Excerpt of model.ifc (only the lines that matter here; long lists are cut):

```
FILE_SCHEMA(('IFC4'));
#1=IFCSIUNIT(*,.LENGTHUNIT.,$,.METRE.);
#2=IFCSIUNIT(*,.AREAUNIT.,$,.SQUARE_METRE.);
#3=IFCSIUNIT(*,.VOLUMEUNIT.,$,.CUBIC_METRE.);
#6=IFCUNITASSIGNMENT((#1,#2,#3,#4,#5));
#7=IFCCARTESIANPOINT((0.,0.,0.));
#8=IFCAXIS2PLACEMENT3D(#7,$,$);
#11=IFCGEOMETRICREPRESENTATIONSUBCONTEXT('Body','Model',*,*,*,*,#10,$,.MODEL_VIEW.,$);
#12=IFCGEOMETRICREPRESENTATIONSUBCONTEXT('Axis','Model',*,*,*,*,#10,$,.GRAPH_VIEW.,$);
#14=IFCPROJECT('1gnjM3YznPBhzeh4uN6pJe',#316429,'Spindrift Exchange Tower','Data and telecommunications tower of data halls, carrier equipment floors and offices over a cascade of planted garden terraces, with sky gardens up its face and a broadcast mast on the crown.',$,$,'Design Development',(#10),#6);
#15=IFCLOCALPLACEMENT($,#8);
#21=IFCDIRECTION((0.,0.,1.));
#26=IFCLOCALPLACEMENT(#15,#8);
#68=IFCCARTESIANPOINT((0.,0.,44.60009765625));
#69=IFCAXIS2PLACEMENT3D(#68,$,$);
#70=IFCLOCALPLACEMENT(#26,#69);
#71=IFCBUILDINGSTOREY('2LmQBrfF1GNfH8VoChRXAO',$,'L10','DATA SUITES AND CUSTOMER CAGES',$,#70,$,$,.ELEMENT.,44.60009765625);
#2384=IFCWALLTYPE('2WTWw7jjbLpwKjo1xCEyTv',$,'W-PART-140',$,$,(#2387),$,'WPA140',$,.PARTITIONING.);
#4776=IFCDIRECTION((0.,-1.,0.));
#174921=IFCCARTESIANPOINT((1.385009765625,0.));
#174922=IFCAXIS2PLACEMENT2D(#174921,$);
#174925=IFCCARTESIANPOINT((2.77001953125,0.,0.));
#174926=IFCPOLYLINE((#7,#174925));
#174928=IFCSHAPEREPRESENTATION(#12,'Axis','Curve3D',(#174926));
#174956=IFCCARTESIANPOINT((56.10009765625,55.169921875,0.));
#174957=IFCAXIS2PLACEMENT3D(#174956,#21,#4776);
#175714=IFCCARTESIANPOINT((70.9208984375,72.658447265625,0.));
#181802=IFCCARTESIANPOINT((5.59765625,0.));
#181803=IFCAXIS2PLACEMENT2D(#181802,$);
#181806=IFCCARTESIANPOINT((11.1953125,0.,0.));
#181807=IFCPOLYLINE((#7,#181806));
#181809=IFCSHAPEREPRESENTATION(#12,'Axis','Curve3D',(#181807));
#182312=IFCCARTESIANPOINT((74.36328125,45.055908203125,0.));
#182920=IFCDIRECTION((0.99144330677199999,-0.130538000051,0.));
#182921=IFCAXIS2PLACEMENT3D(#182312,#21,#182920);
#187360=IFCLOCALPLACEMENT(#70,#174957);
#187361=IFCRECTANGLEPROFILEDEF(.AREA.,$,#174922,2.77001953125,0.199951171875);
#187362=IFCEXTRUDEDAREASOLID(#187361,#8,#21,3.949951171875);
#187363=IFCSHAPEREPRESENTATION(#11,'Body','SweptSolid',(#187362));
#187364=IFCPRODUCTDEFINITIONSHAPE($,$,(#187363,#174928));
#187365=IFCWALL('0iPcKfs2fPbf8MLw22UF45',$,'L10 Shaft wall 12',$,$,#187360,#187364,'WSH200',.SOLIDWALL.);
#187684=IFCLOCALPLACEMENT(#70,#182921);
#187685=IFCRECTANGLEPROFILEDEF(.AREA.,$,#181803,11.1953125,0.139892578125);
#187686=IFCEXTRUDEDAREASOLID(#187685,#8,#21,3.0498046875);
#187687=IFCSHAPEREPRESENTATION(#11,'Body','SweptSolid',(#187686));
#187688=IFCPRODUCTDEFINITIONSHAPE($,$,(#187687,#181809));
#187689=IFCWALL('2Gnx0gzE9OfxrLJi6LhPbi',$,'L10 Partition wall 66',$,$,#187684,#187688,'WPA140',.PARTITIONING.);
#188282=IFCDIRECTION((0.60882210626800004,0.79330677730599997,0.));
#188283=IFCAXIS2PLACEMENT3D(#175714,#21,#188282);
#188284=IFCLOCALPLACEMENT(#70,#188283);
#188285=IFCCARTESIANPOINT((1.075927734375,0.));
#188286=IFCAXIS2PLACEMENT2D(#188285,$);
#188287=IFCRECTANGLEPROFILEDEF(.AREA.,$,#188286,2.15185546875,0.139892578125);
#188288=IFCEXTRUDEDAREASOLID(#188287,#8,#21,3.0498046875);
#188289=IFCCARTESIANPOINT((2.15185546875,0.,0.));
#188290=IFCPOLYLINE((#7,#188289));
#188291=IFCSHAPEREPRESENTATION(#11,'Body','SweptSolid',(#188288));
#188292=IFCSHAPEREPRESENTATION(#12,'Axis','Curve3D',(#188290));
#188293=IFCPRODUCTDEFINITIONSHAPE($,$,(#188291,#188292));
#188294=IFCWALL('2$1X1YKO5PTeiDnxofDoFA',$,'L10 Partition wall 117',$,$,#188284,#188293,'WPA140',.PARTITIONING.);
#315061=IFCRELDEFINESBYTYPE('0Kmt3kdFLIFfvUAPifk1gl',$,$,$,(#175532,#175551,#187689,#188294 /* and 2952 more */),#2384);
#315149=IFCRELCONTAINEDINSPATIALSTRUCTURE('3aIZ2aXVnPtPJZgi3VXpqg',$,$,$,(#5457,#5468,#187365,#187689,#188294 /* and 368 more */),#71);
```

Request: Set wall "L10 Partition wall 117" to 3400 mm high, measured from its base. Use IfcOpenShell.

```python
import ifcopenshell
import ifcopenshell.geom
import ifcopenshell.util.representation
import ifcopenshell.util.shape
import ifcopenshell.util.unit

model = ifcopenshell.open("model.ifc")
unit_scale = ifcopenshell.util.unit.calculate_unit_scale(model)
settings = ifcopenshell.geom.settings()


def volume(element):
    """Net volume in cubic metres, openings subtracted."""
    shape = ifcopenshell.geom.create_shape(settings, element)
    return ifcopenshell.util.shape.get_volume(shape.geometry)


wall = model.by_guid("2$1X1YKO5PTeiDnxofDoFA")
before = volume(wall)

body = ifcopenshell.util.representation.get_representation(wall, "Model", "Body")
solid = body.Items[0]
old_height = solid.Depth
solid.Depth = 3.4 / unit_scale
after = volume(wall)

print(f"height {old_height:g} -> {solid.Depth:g}, volume {before:.3f} -> {after:.3f} m3")

model.write("model_edited.ifc")
```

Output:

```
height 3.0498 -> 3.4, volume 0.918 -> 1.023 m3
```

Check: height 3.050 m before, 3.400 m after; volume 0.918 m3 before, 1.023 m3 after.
